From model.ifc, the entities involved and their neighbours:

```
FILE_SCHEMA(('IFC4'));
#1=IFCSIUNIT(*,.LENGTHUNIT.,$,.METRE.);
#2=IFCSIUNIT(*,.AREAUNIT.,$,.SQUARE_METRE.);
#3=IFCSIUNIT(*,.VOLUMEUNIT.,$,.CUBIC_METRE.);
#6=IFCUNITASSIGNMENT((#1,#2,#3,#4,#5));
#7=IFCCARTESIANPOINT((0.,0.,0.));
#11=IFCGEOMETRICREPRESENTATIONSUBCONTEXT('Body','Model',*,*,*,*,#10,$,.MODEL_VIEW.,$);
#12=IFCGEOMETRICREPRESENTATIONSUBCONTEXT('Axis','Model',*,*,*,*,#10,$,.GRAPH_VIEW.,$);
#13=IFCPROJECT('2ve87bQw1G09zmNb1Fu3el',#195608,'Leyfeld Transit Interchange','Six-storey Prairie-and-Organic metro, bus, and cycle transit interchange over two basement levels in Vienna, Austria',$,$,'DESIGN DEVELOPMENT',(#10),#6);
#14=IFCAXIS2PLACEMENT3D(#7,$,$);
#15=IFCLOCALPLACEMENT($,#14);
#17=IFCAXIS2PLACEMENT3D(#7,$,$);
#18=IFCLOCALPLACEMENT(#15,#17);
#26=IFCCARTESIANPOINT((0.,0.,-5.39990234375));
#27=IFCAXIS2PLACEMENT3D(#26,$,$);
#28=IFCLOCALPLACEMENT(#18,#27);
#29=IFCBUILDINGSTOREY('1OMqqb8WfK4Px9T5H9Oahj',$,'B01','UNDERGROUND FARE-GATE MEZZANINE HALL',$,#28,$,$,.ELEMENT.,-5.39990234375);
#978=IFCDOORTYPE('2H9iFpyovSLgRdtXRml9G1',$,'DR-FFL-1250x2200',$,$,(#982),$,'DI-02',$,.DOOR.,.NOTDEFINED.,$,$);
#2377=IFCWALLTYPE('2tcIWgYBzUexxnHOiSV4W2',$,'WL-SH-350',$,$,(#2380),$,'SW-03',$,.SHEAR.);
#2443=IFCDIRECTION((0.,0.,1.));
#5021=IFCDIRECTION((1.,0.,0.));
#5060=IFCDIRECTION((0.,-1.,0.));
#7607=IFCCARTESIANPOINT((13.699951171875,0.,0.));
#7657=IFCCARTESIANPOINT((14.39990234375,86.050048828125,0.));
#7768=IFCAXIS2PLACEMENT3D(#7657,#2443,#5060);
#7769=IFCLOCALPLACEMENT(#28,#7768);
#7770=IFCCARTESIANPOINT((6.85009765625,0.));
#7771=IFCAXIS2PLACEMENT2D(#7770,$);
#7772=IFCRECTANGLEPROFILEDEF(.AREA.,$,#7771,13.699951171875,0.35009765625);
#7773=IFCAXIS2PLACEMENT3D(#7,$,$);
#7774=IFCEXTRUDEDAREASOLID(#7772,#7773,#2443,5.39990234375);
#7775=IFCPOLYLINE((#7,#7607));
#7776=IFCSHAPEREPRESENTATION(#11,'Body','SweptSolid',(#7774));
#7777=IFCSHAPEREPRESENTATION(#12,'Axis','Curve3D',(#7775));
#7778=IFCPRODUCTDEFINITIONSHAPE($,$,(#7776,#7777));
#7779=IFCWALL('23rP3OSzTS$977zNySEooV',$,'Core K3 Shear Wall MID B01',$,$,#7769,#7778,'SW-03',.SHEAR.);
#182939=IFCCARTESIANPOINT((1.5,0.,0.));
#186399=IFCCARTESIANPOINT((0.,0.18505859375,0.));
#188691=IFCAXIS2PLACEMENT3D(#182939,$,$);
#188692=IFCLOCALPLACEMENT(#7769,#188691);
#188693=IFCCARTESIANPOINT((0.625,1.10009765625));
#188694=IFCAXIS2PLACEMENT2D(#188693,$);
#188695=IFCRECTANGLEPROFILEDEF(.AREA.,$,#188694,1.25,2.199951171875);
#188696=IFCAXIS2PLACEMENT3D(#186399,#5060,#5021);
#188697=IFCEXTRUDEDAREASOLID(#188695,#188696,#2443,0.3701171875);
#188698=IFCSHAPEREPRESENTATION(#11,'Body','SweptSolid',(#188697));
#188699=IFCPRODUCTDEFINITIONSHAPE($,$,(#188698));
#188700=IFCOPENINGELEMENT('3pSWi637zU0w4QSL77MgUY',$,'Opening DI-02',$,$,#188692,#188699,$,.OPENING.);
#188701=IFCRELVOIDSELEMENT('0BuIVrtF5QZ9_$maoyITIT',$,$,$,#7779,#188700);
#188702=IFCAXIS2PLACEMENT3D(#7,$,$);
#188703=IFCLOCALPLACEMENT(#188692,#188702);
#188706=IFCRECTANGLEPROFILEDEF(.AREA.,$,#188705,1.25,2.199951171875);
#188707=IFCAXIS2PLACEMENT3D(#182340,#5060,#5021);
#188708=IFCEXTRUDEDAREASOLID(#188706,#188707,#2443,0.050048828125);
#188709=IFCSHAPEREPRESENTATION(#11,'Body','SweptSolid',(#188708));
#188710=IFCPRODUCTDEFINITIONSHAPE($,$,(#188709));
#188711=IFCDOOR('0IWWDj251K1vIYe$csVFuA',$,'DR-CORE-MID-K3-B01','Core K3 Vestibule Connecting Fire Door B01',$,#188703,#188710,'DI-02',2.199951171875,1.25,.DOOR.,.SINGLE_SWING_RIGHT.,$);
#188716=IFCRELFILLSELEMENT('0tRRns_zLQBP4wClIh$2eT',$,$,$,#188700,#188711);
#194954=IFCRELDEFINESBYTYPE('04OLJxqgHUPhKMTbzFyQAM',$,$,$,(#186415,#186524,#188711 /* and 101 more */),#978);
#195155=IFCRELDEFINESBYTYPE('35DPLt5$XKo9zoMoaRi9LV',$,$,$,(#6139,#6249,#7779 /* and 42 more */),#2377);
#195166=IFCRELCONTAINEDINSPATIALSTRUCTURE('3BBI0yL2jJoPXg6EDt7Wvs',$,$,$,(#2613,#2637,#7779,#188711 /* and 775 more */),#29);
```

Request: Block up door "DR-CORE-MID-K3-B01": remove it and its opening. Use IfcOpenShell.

```python
import ifcopenshell
import ifcopenshell.api.feature
import ifcopenshell.api.root
import ifcopenshell.geom
import ifcopenshell.util.shape

model = ifcopenshell.open("model.ifc")
settings = ifcopenshell.geom.settings()


def volume(element):
    """Net volume in cubic metres, openings subtracted."""
    shape = ifcopenshell.geom.create_shape(settings, element)
    return ifcopenshell.util.shape.get_volume(shape.geometry)


door = model.by_guid("0IWWDj251K1vIYe$csVFuA")
opening = door.FillsVoids[0].RelatingOpeningElement
wall = opening.VoidsElements[0].RelatingBuildingElement
before = volume(wall)

ifcopenshell.api.root.remove_product(model, product=door)
ifcopenshell.api.feature.remove_feature(model, feature=opening)

after = volume(wall)

print(f"wall volume {before:.3f} -> {after:.3f} m3")

model.write("model_rev.ifc")
```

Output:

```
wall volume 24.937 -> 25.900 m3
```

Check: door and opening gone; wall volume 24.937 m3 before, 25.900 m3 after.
